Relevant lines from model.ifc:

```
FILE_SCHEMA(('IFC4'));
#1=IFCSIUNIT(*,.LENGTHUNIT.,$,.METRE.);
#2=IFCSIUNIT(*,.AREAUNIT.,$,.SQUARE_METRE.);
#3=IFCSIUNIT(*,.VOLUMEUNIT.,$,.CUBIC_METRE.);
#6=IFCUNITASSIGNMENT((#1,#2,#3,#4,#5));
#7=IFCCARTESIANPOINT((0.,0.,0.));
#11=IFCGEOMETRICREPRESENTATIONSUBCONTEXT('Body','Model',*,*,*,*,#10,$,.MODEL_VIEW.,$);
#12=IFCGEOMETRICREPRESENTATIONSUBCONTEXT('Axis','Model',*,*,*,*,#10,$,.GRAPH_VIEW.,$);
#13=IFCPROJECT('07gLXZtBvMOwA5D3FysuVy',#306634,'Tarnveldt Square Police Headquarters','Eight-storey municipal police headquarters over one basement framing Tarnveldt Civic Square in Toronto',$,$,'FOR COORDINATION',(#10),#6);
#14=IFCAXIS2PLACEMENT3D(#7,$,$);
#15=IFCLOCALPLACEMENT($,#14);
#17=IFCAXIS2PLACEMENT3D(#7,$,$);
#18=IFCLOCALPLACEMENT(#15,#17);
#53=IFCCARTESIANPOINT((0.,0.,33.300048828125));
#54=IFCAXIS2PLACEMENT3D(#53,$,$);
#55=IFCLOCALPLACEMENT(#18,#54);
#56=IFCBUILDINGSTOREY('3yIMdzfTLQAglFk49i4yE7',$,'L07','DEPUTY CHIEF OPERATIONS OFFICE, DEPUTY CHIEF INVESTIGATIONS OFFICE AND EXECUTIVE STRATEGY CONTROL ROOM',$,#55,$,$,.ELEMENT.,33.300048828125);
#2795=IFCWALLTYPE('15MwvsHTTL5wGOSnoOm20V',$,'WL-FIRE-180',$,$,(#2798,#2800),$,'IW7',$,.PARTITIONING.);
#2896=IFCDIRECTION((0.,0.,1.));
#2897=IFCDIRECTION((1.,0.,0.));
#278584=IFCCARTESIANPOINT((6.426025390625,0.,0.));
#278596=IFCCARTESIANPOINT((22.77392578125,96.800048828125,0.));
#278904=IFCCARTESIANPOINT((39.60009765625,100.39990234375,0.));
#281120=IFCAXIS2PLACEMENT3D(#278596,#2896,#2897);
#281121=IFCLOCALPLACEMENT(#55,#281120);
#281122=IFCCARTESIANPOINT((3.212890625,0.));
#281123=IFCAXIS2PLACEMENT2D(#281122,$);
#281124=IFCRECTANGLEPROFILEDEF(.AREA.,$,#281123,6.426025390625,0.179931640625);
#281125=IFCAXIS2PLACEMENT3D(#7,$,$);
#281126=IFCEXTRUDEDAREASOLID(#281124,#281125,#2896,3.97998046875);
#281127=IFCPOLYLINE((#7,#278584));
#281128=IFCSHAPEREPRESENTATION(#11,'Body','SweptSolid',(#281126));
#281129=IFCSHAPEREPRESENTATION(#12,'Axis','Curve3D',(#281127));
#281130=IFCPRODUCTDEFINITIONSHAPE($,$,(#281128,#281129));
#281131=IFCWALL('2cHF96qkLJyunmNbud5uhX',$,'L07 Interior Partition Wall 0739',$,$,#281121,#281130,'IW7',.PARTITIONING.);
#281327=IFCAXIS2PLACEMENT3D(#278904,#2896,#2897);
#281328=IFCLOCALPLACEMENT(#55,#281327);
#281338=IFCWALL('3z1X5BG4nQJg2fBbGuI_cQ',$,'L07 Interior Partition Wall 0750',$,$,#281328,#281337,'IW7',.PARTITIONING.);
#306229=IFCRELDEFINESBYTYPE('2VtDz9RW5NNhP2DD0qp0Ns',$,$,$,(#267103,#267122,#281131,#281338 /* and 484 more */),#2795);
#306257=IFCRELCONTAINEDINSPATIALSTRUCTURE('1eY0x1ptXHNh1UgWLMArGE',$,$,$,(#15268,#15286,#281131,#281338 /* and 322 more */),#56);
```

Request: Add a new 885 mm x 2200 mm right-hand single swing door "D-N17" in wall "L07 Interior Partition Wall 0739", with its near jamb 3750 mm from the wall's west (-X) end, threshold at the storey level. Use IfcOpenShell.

```python
import numpy as np
import ifcopenshell
import ifcopenshell.api.feature
import ifcopenshell.api.geometry
import ifcopenshell.api.root
import ifcopenshell.api.spatial
import ifcopenshell.geom
import ifcopenshell.util.element
import ifcopenshell.util.placement
import ifcopenshell.util.representation
import ifcopenshell.util.shape
import ifcopenshell.util.unit

model = ifcopenshell.open("model.ifc")
unit_scale = ifcopenshell.util.unit.calculate_unit_scale(model)
settings = ifcopenshell.geom.settings()


def volume(element):
    """Net volume in cubic metres, openings subtracted."""
    shape = ifcopenshell.geom.create_shape(settings, element)
    return ifcopenshell.util.shape.get_volume(shape.geometry)


wall = model.by_guid("2cHF96qkLJyunmNbud5uhX")
storey = ifcopenshell.util.element.get_container(wall, ifc_class="IfcBuildingStorey")
context = ifcopenshell.util.representation.get_context(model, "Model", "Body", "MODEL_VIEW")
before = volume(wall)

width, height, from_end, sill = 0.885, 2.2, 3.75, 0.0  # metres

# The wall runs along its own X axis, and the end named is its -X end.
wall_shape = ifcopenshell.geom.create_shape(settings, wall)
x, y, z = ifcopenshell.util.shape.get_vertices(wall_shape.geometry).T
start = x.min() + from_end
face, thickness = float(y.min()), float(y.max() - y.min())
wall_matrix = ifcopenshell.util.placement.get_local_placement(wall.ObjectPlacement)
level = ifcopenshell.util.placement.get_local_placement(storey.ObjectPlacement)[2, 3]


def in_wall(x, y):
    """Placement at x, y metres in the wall's axes, at sill height."""
    matrix = wall_matrix.copy()
    matrix[:, 3] = wall_matrix @ np.array([x / unit_scale, y / unit_scale, 0.0, 1.0])
    matrix[2, 3] = level + sill / unit_scale
    return matrix


# Opening: a box that overshoots both wall faces by 50 mm.
opening = ifcopenshell.api.root.create_entity(model, ifc_class="IfcOpeningElement", predefined_type="OPENING")
box = ifcopenshell.api.geometry.add_wall_representation(
    model, context=context, length=width, height=height, thickness=thickness + 0.1
)
ifcopenshell.api.geometry.assign_representation(model, product=opening, representation=box)
ifcopenshell.api.geometry.edit_object_placement(model, product=opening, matrix=in_wall(start, face - 0.05), is_si=False)
ifcopenshell.api.feature.add_feature(model, feature=opening, element=wall)

door = ifcopenshell.api.root.create_entity(model, ifc_class="IfcDoor", name="D-N17", predefined_type="DOOR")
door.OverallWidth, door.OverallHeight = width / unit_scale, height / unit_scale
door.OperationType = "SINGLE_SWING_RIGHT"
body = ifcopenshell.api.geometry.add_door_representation(
    model,
    context=context,
    overall_width=door.OverallWidth,
    overall_height=door.OverallHeight,
    operation_type="SINGLE_SWING_RIGHT",
    lining_properties={"LiningDepth": thickness / unit_scale, "ThresholdDepth": thickness / unit_scale},
)
ifcopenshell.api.geometry.assign_representation(model, product=door, representation=body)
ifcopenshell.api.spatial.assign_container(model, products=[door], relating_structure=storey)
ifcopenshell.api.feature.add_filling(model, opening=opening, element=door)

# The lining spans the wall, so the door starts at the wall face.
ifcopenshell.api.geometry.edit_object_placement(model, product=door, matrix=in_wall(start, face), is_si=False)

after = volume(wall)

print(f"wall volume {before:.3f} -> {after:.3f} m3")

model.write("model_rev.ifc")
```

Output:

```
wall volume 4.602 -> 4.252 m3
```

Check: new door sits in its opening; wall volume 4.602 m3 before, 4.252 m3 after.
